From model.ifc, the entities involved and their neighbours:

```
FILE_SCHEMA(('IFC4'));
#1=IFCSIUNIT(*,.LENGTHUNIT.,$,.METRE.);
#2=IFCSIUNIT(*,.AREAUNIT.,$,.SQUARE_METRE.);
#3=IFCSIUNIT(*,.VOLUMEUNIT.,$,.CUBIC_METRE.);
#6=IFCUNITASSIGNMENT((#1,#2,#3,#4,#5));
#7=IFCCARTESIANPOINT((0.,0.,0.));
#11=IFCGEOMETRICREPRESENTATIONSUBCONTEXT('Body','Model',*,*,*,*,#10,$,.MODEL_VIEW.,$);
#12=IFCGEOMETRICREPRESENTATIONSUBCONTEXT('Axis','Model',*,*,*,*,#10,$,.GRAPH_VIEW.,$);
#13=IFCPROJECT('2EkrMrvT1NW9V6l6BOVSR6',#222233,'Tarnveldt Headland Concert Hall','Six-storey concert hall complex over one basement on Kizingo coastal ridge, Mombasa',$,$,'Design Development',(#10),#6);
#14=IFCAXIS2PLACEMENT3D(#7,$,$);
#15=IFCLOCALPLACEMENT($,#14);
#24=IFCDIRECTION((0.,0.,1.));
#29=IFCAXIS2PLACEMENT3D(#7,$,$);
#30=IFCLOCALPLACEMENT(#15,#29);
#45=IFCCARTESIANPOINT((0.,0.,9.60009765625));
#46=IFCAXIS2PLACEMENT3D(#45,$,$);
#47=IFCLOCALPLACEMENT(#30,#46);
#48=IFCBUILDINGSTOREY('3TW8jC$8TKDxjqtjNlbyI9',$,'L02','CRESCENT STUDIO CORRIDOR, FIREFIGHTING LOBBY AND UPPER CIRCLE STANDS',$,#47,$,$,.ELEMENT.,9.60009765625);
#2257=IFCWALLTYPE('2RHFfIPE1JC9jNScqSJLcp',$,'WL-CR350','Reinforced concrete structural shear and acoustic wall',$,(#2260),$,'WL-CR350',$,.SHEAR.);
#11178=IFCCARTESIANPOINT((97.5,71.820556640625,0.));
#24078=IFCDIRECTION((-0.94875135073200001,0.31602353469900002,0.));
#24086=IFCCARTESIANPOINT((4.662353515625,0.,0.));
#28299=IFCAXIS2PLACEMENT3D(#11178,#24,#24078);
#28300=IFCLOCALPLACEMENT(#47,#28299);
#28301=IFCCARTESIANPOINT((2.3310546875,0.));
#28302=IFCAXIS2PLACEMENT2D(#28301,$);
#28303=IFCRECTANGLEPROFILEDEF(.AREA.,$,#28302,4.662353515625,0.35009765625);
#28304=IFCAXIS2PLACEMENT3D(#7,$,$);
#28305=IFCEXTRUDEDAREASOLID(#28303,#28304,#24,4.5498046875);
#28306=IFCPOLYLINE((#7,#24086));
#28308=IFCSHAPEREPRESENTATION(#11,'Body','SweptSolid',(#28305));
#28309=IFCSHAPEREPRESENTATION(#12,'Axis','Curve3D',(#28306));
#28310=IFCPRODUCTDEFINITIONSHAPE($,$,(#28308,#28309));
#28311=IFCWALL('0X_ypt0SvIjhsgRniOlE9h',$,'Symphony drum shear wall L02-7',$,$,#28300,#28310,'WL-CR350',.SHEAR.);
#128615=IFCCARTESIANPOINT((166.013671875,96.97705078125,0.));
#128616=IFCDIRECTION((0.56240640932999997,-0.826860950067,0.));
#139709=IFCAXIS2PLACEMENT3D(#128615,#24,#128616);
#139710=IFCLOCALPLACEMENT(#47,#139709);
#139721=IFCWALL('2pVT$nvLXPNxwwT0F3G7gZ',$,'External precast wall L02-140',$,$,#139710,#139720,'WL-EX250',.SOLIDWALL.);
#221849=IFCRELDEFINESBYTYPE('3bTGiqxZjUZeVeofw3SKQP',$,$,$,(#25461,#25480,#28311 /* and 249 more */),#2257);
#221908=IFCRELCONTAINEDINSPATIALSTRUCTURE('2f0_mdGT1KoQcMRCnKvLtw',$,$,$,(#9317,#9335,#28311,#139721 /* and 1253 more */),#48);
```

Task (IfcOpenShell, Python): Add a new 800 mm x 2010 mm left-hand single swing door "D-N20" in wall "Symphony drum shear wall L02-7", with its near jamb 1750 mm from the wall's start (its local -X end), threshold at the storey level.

```python
import numpy as np
import ifcopenshell
import ifcopenshell.api.feature
import ifcopenshell.api.geometry
import ifcopenshell.api.root
import ifcopenshell.api.spatial
import ifcopenshell.geom
import ifcopenshell.util.element
import ifcopenshell.util.placement
import ifcopenshell.util.representation
import ifcopenshell.util.shape
import ifcopenshell.util.unit

model = ifcopenshell.open("model.ifc")
unit_scale = ifcopenshell.util.unit.calculate_unit_scale(model)
settings = ifcopenshell.geom.settings()


def volume(element):
    """Net volume in cubic metres, openings subtracted."""
    shape = ifcopenshell.geom.create_shape(settings, element)
    return ifcopenshell.util.shape.get_volume(shape.geometry)


wall = model.by_id(28311)
storey = ifcopenshell.util.element.get_container(wall, ifc_class="IfcBuildingStorey")
context = ifcopenshell.util.representation.get_context(model, "Model", "Body", "MODEL_VIEW")
before = volume(wall)

width, height, from_end, sill = 0.8, 2.01, 1.75, 0.0  # metres

# The wall runs along its own X axis, and the end named is its -X end.
wall_shape = ifcopenshell.geom.create_shape(settings, wall)
x, y, z = ifcopenshell.util.shape.get_vertices(wall_shape.geometry).T
start = x.min() + from_end
face, thickness = float(y.min()), float(y.max() - y.min())
wall_matrix = ifcopenshell.util.placement.get_local_placement(wall.ObjectPlacement)
level = ifcopenshell.util.placement.get_local_placement(storey.ObjectPlacement)[2, 3]


def in_wall(x, y):
    """Placement at x, y metres in the wall's axes, at sill height."""
    matrix = wall_matrix.copy()
    matrix[:, 3] = wall_matrix @ np.array([x / unit_scale, y / unit_scale, 0.0, 1.0])
    matrix[2, 3] = level + sill / unit_scale
    return matrix


# Opening: a box that overshoots both wall faces by 50 mm.
opening = ifcopenshell.api.root.create_entity(model, ifc_class="IfcOpeningElement", predefined_type="OPENING")
box = ifcopenshell.api.geometry.add_wall_representation(
    model, context=context, length=width, height=height, thickness=thickness + 0.1
)
ifcopenshell.api.geometry.assign_representation(model, product=opening, representation=box)
ifcopenshell.api.geometry.edit_object_placement(model, product=opening, matrix=in_wall(start, face - 0.05), is_si=False)
ifcopenshell.api.feature.add_feature(model, feature=opening, element=wall)

door = ifcopenshell.api.root.create_entity(model, ifc_class="IfcDoor", name="D-N20", predefined_type="DOOR")
door.OverallWidth, door.OverallHeight = width / unit_scale, height / unit_scale
door.OperationType = "SINGLE_SWING_LEFT"
body = ifcopenshell.api.geometry.add_door_representation(
    model,
    context=context,
    overall_width=door.OverallWidth,
    overall_height=door.OverallHeight,
    operation_type="SINGLE_SWING_LEFT",
    lining_properties={"LiningDepth": thickness / unit_scale, "ThresholdDepth": thickness / unit_scale},
)
ifcopenshell.api.geometry.assign_representation(model, product=door, representation=body)
ifcopenshell.api.spatial.assign_container(model, products=[door], relating_structure=storey)
ifcopenshell.api.feature.add_filling(model, opening=opening, element=door)

# The lining spans the wall, so the door starts at the wall face.
ifcopenshell.api.geometry.edit_object_placement(model, product=door, matrix=in_wall(start, face), is_si=False)

after = volume(wall)

print(f"wall volume {before:.3f} -> {after:.3f} m3")

model.write("model_rev.ifc")
```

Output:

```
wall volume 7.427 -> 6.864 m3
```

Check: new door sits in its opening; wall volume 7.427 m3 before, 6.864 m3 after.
